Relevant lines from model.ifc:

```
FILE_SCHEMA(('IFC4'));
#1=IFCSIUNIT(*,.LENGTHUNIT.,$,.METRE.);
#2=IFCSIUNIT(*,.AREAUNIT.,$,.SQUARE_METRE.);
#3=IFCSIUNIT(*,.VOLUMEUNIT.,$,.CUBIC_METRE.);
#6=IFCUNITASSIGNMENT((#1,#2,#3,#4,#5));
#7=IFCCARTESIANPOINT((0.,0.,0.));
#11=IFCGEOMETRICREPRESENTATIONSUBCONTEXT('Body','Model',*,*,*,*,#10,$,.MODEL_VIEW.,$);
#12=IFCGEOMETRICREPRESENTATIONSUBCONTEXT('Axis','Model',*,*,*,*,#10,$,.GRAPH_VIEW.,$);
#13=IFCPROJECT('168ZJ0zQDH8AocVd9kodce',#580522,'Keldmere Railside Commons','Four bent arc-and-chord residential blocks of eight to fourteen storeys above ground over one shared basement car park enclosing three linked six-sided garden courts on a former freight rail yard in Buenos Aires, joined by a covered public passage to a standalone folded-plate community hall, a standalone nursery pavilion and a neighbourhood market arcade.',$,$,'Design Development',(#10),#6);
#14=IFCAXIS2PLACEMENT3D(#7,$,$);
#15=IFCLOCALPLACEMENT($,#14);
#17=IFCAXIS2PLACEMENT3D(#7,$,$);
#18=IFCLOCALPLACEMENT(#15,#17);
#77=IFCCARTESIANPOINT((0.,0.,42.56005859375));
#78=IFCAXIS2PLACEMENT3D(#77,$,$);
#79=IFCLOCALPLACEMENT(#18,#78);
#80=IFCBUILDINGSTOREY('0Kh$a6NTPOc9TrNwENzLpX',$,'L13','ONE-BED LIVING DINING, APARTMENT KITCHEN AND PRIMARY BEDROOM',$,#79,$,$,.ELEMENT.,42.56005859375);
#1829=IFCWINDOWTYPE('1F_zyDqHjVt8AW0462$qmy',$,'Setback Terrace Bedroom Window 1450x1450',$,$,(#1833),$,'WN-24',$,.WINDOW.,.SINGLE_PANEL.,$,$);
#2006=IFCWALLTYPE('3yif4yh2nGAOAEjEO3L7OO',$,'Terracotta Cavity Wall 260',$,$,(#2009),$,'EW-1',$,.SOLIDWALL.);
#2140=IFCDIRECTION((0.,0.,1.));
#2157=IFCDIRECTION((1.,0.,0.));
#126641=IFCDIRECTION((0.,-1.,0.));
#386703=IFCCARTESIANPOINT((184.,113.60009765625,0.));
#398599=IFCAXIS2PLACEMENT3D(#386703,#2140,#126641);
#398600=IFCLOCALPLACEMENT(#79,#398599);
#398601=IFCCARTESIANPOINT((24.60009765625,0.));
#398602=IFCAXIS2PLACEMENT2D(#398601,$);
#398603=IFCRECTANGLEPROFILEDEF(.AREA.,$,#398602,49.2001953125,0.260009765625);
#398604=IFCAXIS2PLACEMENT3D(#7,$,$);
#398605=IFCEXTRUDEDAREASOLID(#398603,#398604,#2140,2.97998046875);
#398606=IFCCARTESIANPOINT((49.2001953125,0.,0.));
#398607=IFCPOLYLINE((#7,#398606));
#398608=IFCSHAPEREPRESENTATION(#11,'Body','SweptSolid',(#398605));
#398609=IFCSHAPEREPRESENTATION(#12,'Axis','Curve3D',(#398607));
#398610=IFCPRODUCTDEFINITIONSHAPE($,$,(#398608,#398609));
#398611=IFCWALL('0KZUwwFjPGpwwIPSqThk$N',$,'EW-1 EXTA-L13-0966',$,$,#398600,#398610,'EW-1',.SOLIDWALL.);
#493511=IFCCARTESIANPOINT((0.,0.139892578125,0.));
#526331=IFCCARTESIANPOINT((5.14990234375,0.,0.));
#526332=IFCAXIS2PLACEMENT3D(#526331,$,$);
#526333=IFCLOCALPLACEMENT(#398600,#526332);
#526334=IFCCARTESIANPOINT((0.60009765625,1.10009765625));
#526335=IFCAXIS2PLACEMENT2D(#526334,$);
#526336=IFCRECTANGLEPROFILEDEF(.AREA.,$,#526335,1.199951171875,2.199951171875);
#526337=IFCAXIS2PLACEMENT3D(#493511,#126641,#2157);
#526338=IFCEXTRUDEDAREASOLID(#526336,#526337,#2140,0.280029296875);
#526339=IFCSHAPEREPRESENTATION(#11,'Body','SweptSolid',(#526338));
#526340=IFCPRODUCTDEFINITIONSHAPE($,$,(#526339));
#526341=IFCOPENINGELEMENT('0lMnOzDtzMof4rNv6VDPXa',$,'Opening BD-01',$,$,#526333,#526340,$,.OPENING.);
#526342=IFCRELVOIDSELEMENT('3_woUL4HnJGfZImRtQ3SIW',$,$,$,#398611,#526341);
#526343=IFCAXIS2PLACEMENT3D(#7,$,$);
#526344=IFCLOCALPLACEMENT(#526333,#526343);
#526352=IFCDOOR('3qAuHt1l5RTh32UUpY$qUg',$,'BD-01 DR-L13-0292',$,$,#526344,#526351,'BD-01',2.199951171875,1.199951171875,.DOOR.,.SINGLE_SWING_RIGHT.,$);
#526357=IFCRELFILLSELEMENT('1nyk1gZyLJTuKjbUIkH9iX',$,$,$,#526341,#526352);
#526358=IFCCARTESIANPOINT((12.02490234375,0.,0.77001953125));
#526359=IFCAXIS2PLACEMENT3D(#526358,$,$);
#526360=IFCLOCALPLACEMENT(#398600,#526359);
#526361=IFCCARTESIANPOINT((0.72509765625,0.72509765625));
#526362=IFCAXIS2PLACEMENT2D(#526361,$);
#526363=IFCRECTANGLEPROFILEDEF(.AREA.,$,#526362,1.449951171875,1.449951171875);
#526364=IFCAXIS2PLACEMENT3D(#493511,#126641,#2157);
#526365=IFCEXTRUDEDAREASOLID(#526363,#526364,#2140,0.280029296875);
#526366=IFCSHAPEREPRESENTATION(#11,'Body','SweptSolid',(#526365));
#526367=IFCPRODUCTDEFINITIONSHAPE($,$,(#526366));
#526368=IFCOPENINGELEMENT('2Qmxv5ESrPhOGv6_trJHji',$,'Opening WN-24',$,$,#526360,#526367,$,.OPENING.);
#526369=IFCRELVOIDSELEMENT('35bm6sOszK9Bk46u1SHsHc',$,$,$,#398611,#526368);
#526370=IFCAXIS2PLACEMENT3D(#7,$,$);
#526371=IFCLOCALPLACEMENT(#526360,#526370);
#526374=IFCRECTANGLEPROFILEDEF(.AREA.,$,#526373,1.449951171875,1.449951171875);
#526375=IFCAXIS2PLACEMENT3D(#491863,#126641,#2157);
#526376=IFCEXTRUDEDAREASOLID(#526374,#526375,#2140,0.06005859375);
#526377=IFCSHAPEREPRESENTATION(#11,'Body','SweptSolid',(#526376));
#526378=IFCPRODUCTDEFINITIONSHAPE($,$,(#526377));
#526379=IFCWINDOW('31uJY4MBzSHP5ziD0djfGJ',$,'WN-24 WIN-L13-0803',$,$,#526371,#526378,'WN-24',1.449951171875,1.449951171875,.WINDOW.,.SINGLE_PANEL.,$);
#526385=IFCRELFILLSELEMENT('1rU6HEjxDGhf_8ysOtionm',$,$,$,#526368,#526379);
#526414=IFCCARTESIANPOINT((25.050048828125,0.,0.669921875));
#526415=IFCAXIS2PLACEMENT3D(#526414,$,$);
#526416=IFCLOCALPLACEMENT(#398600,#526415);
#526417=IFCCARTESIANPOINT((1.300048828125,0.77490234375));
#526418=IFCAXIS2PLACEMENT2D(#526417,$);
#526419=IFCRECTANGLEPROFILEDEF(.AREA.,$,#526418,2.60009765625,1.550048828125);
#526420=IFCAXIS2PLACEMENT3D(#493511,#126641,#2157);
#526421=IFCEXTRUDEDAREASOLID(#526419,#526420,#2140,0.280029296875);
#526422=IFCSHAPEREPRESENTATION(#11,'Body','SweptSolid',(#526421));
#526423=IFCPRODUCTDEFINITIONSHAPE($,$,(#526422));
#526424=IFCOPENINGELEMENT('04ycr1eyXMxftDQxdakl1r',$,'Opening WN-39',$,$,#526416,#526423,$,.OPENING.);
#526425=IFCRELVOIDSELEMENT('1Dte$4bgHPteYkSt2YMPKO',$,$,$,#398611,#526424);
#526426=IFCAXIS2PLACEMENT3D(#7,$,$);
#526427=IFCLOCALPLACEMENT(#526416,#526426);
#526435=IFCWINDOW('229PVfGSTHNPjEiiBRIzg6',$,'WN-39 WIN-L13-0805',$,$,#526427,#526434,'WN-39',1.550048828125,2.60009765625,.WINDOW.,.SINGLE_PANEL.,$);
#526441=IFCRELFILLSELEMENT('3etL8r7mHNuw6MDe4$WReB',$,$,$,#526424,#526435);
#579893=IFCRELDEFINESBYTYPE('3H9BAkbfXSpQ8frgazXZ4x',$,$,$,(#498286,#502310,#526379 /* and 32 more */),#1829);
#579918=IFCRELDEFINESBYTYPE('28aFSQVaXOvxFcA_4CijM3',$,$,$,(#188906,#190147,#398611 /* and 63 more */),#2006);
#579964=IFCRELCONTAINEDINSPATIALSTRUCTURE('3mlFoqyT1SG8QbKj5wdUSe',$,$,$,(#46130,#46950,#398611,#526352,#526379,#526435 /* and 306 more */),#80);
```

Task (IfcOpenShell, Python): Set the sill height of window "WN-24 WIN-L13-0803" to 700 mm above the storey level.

```python
import numpy as np
import ifcopenshell
import ifcopenshell.api.geometry
import ifcopenshell.geom
import ifcopenshell.util.element
import ifcopenshell.util.placement
import ifcopenshell.util.shape
import ifcopenshell.util.unit

model = ifcopenshell.open("model.ifc")
unit_scale = ifcopenshell.util.unit.calculate_unit_scale(model)

window = model.by_guid("31uJY4MBzSHP5ziD0djfGJ")
opening = window.FillsVoids[0].RelatingOpeningElement
storey = ifcopenshell.util.element.get_container(window, ifc_class="IfcBuildingStorey")
level = ifcopenshell.util.placement.get_local_placement(storey.ObjectPlacement)[2, 3]

# The opening's origin need not be at the sill, so measure its lowest point.
shape = ifcopenshell.geom.create_shape(ifcopenshell.geom.settings(), opening)
bottom = ifcopenshell.util.shape.get_shape_bottom_elevation(shape, shape.geometry) / unit_scale
dz = level + 0.7 - bottom

shift = np.array([0.0, 0.0, dz])
# The window is placed relative to its opening, so it follows when the opening moves.
matrix = ifcopenshell.util.placement.get_local_placement(opening.ObjectPlacement)
matrix[:3, 3] += shift
ifcopenshell.api.geometry.edit_object_placement(
    model, product=opening, matrix=matrix, is_si=False, should_transform_children=True
)

print(f"moved by {dz * unit_scale:+.3f} m")

model.write("model_rev.ifc")
```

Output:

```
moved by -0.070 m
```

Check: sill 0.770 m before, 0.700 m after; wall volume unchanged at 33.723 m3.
